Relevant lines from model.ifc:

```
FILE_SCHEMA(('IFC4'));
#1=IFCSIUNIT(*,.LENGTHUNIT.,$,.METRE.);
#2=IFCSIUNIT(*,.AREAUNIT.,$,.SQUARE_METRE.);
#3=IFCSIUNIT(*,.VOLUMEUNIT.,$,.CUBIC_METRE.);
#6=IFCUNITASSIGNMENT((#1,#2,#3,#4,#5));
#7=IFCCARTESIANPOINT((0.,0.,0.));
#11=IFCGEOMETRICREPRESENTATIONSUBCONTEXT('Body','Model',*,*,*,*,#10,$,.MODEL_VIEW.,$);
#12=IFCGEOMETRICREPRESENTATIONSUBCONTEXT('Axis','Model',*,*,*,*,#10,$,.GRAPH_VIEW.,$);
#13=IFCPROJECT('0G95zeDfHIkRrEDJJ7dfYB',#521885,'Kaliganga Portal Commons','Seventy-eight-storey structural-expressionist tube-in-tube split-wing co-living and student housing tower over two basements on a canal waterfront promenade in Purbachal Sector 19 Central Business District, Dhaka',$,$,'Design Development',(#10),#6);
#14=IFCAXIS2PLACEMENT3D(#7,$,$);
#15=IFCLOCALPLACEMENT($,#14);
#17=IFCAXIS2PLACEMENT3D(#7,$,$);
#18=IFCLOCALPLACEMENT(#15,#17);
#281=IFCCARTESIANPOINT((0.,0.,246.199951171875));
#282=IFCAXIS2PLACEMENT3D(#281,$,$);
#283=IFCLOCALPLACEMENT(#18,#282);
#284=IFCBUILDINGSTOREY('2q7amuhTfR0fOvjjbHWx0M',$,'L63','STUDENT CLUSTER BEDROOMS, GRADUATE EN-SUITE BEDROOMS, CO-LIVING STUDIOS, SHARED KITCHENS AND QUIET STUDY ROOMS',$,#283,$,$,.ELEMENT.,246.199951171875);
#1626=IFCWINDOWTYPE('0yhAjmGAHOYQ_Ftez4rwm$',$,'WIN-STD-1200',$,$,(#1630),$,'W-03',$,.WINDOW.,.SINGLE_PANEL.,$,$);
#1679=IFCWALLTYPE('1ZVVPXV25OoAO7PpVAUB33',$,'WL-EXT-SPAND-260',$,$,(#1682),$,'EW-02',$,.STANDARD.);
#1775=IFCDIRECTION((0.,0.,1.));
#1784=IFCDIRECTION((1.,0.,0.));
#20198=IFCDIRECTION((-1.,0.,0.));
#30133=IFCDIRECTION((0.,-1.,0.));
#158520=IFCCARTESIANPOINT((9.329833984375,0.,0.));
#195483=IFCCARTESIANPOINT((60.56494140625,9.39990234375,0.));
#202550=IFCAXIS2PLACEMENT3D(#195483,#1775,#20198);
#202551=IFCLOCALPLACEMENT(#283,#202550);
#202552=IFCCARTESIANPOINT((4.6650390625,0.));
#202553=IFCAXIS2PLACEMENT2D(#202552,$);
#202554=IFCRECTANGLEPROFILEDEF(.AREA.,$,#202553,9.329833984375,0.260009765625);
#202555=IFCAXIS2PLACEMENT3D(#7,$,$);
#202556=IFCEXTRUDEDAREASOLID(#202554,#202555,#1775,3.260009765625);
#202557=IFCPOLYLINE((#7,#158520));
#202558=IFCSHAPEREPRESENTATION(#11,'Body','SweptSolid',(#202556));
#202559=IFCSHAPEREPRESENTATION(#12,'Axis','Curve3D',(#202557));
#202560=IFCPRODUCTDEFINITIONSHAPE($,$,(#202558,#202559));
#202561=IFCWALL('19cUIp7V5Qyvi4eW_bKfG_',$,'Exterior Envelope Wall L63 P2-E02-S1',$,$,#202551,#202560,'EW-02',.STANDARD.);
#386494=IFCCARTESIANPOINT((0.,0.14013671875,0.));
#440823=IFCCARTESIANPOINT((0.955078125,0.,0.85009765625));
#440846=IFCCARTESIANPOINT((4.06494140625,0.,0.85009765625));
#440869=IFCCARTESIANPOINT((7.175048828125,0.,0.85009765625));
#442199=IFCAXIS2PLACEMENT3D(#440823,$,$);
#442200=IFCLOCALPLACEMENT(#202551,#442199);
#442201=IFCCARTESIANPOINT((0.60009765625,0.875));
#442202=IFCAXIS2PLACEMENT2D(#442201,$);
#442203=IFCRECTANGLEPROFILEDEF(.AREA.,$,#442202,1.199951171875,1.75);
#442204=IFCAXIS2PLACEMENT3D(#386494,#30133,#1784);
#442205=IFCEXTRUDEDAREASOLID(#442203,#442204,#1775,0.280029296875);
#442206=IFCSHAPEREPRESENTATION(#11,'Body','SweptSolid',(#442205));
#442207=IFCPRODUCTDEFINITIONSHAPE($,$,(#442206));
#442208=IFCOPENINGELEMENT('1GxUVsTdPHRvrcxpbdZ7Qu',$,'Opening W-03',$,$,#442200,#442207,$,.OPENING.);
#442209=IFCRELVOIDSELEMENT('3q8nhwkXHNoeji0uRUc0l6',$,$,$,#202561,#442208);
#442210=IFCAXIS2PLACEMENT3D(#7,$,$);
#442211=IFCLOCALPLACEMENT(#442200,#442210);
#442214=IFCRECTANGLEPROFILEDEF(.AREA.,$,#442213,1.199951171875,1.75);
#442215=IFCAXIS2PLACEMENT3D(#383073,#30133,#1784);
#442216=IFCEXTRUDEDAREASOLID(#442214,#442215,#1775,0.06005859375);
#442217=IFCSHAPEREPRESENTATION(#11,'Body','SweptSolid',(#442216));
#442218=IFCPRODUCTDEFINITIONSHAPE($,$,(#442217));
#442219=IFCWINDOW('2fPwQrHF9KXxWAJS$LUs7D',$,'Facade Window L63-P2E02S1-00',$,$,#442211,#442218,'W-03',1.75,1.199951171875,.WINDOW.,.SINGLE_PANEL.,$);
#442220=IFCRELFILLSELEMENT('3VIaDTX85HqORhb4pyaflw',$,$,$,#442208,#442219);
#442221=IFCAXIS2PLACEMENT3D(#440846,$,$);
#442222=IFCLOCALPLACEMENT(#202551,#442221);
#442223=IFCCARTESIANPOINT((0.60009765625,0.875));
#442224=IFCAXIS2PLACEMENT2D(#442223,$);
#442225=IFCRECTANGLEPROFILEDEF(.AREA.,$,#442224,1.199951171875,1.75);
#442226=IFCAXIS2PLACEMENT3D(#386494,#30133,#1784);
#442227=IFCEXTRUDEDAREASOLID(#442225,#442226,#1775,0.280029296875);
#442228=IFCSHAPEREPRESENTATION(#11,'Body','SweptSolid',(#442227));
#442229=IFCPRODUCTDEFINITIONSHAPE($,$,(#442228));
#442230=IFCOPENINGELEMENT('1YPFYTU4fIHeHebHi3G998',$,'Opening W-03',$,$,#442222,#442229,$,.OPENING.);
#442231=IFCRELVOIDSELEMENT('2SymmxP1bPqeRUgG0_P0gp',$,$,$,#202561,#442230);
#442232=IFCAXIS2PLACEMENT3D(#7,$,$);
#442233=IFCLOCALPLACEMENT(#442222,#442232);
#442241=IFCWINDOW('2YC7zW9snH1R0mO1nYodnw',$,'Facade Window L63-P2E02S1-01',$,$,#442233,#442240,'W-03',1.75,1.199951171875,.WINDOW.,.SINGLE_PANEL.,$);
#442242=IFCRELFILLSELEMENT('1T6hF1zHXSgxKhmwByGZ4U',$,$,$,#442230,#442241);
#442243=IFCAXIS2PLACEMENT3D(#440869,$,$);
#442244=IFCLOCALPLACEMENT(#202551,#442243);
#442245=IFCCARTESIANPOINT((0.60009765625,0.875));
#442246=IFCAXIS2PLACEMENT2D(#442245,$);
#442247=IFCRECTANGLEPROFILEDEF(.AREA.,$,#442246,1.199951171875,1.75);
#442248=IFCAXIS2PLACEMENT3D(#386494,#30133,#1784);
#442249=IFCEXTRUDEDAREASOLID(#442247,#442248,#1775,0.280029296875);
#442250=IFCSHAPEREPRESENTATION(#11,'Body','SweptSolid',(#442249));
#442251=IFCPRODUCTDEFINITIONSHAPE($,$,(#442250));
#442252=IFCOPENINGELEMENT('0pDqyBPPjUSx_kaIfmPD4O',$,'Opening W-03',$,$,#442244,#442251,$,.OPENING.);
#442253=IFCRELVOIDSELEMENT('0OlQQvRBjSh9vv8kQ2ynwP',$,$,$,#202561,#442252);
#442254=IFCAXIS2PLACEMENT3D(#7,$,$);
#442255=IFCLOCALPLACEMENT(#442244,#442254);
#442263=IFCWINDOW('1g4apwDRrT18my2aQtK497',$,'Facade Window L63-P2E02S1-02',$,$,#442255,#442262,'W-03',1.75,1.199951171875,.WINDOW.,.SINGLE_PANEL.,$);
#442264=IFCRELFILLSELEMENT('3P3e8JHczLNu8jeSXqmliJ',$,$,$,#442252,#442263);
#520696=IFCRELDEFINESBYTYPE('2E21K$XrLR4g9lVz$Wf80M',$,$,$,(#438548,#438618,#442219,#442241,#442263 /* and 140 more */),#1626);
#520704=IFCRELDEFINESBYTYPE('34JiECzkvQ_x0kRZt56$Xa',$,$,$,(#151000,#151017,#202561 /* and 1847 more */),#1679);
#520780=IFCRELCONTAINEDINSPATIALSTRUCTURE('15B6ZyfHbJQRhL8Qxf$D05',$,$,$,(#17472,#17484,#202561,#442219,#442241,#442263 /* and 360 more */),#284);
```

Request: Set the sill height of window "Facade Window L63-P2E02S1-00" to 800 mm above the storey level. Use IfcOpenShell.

```python
import numpy as np
import ifcopenshell
import ifcopenshell.api.geometry
import ifcopenshell.geom
import ifcopenshell.util.element
import ifcopenshell.util.placement
import ifcopenshell.util.shape
import ifcopenshell.util.unit

model = ifcopenshell.open("model.ifc")
unit_scale = ifcopenshell.util.unit.calculate_unit_scale(model)

window = model.by_guid("2fPwQrHF9KXxWAJS$LUs7D")
opening = window.FillsVoids[0].RelatingOpeningElement
storey = ifcopenshell.util.element.get_container(window, ifc_class="IfcBuildingStorey")
level = ifcopenshell.util.placement.get_local_placement(storey.ObjectPlacement)[2, 3]

# The opening's origin need not be at the sill, so measure its lowest point.
shape = ifcopenshell.geom.create_shape(ifcopenshell.geom.settings(), opening)
bottom = ifcopenshell.util.shape.get_shape_bottom_elevation(shape, shape.geometry) / unit_scale
dz = level + 0.8 / unit_scale - bottom

shift = np.array([0.0, 0.0, dz])
# The window is placed relative to its opening, so it follows when the opening moves.
matrix = ifcopenshell.util.placement.get_local_placement(opening.ObjectPlacement)
matrix[:3, 3] += shift
ifcopenshell.api.geometry.edit_object_placement(
    model, product=opening, matrix=matrix, is_si=False, should_transform_children=True
)

print(f"moved by {dz * unit_scale:+.3f} m")

model.write("model_updated.ifc")
```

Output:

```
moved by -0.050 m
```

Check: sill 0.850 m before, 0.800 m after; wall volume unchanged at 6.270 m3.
